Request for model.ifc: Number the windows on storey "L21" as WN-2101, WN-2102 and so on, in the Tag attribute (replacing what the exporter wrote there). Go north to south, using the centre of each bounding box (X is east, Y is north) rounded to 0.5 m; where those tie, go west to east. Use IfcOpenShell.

First a look at what the model holds.

```python
import ifcopenshell
import ifcopenshell.util.element
import ifcopenshell.util.placement

model = ifcopenshell.open("model.ifc")
print(model.schema)
storey = next(s for s in model.by_type("IfcBuildingStorey") if s.Name == "L21")
windows = [e for e in ifcopenshell.util.element.get_decomposition(storey) if e.is_a("IfcWindow")]
for e in sorted(windows, key=lambda e: e.id()):
    origin = ifcopenshell.util.placement.get_local_placement(e.ObjectPlacement)[:3, 3]
    print(e.id(), e.Tag, e.Name, origin.round(2) + 0.0, sep=" | ")
```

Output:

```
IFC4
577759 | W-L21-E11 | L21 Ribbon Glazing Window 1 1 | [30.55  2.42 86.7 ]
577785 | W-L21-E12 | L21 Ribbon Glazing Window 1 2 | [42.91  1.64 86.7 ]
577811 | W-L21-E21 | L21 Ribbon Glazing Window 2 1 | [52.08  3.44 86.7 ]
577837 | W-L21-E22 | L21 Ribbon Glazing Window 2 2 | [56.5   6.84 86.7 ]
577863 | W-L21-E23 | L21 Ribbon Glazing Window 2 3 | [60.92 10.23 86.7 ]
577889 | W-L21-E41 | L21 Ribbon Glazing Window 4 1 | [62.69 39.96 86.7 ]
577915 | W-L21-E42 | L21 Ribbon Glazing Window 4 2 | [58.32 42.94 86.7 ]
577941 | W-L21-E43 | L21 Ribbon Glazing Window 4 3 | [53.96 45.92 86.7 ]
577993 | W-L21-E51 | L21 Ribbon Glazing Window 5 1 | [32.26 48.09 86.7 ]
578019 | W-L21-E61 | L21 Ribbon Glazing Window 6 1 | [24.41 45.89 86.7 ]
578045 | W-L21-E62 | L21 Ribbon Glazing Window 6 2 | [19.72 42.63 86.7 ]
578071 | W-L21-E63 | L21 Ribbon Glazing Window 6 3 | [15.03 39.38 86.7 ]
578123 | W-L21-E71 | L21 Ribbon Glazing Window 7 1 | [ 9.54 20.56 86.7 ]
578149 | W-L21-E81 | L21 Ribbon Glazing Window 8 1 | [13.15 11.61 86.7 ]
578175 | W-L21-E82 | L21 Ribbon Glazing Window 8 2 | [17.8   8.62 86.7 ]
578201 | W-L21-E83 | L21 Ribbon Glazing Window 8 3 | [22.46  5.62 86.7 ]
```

```python
import ifcopenshell
import ifcopenshell.geom
import ifcopenshell.util.element
import ifcopenshell.util.shape

model = ifcopenshell.open("model.ifc")
settings = ifcopenshell.geom.settings()
settings.set("use-world-coords", True)


def centre(element):
    shape = ifcopenshell.geom.create_shape(settings, element)
    return ifcopenshell.util.shape.get_bbox_centroid(shape.geometry)


storey = next(s for s in model.by_type("IfcBuildingStorey") if s.Name == "L21")
windows = [e for e in ifcopenshell.util.element.get_decomposition(storey) if e.is_a("IfcWindow")]

# Insertion points can sit at a corner or the storey origin, so sort by the geometry (in metres).
centres = {e: centre(e) for e in windows}
windows.sort(key=lambda e: (-round(centres[e][1] / 0.5), centres[e][0]))

for i, e in enumerate(windows, start=1):
    number = f"WN-21{i:02d}"
    e.Tag = number
    print(e.id(), number)

model.write("model-out.ifc")
```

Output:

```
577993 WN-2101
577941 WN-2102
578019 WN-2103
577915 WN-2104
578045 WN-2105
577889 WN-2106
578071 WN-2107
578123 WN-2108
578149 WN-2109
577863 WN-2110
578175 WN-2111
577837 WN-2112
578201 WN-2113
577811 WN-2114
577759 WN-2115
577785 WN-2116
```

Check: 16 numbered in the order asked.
